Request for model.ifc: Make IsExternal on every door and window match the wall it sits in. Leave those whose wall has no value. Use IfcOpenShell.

First a look at what the model holds.

```python
import ifcopenshell
import ifcopenshell.util.element

model = ifcopenshell.open("model.ifc")
print(model.schema)
seen = {}
for e in model.by_type("IfcDoor") + model.by_type("IfcWindow"):
    if not e.FillsVoids:
        continue
    host = e.FillsVoids[0].RelatingOpeningElement.VoidsElements[0].RelatingBuildingElement
    own = ifcopenshell.util.element.get_pset(e, f"Pset_{e.is_a()[3:].removesuffix('StandardCase')}Common", "IsExternal")
    wall = ifcopenshell.util.element.get_pset(host, "Pset_WallCommon", "IsExternal")
    seen[e.is_a(), own, wall] = seen.get((e.is_a(), own, wall), 0) + 1
for (cls, own, wall), count in sorted(seen.items(), key=str):
    print(count, cls, "IsExternal:", own, "| host wall:", wall)
```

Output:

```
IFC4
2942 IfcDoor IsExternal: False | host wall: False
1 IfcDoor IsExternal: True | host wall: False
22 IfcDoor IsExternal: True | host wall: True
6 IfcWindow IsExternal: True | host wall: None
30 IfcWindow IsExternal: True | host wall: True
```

```python
import ifcopenshell
import ifcopenshell.api.pset
import ifcopenshell.util.element

model = ifcopenshell.open("model.ifc")

count = 0
for ifc_class, pset_name in (("IfcDoor", "Pset_DoorCommon"), ("IfcWindow", "Pset_WindowCommon")):
    for e in model.by_type(ifc_class):
        if not e.FillsVoids:
            continue
        host = e.FillsVoids[0].RelatingOpeningElement.VoidsElements[0].RelatingBuildingElement
        external = ifcopenshell.util.element.get_pset(host, "Pset_WallCommon", "IsExternal")
        if external is None or ifcopenshell.util.element.get_pset(e, pset_name, "IsExternal") == external:
            continue
        found = ifcopenshell.util.element.get_pset(e, pset_name, should_inherit=False)
        if found:
            pset = model.by_id(found["id"])
            if len(ifcopenshell.util.element.get_elements_by_pset(pset)) > 1:
                pset = ifcopenshell.api.pset.unshare_pset(model, products=[e], pset=pset)[0]
        else:
            pset = ifcopenshell.api.pset.add_pset(model, product=e, name=pset_name)
        ifcopenshell.api.pset.edit_pset(model, pset=pset, properties={"IsExternal": external})
        count += 1

print(count, "updated")

model.write("model_updated.ifc")
```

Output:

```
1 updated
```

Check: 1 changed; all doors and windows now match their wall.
